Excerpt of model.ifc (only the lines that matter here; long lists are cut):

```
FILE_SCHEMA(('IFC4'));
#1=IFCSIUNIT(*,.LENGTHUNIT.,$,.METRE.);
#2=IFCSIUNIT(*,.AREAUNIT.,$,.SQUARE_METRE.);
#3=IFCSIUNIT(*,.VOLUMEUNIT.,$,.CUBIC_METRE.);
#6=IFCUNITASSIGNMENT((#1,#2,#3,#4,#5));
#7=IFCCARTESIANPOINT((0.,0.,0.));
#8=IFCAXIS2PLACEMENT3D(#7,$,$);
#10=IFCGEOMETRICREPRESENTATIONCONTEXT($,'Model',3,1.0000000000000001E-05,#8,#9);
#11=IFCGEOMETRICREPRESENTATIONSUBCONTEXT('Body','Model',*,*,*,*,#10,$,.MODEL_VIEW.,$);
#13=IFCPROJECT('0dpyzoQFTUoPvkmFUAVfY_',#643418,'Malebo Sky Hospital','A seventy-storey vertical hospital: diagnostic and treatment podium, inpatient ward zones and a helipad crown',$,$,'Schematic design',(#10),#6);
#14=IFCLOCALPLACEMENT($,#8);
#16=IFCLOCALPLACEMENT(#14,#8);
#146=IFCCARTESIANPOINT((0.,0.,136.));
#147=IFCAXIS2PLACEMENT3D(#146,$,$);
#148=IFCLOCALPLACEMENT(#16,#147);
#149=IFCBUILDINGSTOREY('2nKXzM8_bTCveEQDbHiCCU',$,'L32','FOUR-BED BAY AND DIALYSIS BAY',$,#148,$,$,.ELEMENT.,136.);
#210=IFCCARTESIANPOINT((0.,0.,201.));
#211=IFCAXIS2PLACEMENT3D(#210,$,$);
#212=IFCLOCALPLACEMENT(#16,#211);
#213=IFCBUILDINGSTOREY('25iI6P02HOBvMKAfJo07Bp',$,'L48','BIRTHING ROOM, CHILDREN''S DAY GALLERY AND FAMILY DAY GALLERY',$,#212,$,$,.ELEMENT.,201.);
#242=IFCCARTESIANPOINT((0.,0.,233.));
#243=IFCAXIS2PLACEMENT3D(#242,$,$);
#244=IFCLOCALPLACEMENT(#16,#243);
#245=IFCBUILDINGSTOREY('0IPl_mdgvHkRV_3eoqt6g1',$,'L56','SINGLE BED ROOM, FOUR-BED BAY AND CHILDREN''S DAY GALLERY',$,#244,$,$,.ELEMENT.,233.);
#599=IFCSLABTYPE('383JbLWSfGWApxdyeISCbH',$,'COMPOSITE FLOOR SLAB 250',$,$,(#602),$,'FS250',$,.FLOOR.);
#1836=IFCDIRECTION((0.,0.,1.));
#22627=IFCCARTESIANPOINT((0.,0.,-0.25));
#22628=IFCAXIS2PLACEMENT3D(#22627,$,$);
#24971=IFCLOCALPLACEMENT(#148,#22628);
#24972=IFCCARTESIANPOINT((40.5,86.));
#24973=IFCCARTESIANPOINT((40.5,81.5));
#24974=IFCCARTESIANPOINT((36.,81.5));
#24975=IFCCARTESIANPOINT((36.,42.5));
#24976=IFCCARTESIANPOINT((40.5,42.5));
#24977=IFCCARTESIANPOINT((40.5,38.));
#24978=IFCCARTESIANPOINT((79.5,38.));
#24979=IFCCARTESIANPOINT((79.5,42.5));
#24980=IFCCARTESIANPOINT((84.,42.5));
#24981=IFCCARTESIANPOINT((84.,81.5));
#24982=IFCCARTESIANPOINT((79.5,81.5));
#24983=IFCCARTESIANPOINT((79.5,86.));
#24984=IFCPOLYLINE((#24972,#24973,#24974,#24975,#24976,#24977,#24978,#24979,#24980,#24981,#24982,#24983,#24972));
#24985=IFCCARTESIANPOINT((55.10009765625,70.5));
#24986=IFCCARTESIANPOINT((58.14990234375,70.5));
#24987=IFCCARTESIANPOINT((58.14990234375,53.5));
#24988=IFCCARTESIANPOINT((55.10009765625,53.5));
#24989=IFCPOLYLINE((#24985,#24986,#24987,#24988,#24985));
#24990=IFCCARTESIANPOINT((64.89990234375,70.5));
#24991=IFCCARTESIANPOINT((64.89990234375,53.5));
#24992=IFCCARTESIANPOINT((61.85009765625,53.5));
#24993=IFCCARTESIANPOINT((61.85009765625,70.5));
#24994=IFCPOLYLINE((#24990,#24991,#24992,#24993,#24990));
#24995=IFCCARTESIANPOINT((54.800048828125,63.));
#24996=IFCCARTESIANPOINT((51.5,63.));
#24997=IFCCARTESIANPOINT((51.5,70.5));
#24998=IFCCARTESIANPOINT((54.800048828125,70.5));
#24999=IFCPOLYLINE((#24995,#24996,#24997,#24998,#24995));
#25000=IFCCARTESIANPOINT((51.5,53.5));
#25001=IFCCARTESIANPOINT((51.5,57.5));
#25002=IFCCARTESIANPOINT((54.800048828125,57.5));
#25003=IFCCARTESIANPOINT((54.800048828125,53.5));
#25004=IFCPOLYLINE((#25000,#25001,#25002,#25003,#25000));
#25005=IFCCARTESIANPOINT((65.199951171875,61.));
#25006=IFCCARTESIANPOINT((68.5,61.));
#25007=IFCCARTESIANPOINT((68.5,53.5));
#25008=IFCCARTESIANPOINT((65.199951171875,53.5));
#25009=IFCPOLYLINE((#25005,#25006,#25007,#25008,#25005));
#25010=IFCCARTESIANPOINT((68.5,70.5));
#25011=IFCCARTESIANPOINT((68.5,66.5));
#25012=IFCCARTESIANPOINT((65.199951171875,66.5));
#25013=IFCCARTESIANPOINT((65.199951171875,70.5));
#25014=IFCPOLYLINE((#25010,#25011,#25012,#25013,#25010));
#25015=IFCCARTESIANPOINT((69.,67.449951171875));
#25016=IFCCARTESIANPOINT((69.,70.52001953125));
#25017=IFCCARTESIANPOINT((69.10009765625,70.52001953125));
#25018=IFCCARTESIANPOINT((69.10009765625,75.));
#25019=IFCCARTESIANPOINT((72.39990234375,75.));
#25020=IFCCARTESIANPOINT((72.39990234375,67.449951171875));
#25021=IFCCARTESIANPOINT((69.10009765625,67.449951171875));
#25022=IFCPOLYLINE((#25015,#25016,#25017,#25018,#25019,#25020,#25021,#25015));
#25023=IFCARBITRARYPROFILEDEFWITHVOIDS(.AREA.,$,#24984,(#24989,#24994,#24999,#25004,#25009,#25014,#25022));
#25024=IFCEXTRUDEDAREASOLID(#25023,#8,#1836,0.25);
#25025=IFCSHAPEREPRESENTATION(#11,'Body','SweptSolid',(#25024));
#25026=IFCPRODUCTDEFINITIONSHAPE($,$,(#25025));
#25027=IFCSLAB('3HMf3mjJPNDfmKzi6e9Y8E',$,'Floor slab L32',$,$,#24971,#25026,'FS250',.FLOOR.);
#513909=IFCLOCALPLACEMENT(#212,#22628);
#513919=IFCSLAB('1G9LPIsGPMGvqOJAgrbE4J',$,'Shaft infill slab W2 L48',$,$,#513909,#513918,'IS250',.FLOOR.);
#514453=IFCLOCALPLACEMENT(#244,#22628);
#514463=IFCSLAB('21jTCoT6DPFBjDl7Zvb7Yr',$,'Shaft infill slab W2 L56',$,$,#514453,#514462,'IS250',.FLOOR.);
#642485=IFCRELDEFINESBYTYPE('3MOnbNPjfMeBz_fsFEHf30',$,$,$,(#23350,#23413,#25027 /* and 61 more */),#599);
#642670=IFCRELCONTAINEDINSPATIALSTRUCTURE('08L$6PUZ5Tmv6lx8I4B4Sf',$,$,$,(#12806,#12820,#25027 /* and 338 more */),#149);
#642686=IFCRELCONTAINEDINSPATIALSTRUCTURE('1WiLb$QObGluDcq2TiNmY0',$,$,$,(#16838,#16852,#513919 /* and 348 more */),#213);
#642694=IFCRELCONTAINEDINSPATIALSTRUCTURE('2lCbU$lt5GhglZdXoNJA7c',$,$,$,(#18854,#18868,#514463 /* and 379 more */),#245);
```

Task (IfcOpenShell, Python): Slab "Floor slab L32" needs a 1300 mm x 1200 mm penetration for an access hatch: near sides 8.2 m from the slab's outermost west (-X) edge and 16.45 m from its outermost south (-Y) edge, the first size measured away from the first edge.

```python
import numpy as np
import ifcopenshell
import ifcopenshell.api.feature
import ifcopenshell.api.geometry
import ifcopenshell.api.root
import ifcopenshell.geom
import ifcopenshell.util.placement
import ifcopenshell.util.representation
import ifcopenshell.util.shape
import ifcopenshell.util.unit

model = ifcopenshell.open("model.ifc")
unit_scale = ifcopenshell.util.unit.calculate_unit_scale(model)
settings = ifcopenshell.geom.settings()


def volume(element):
    """Net volume in cubic metres, openings subtracted."""
    shape = ifcopenshell.geom.create_shape(settings, element)
    return ifcopenshell.util.shape.get_volume(shape.geometry)


slab = model.by_guid("3HMf3mjJPNDfmKzi6e9Y8E")
before = volume(slab)

# Extent in the slab's own axes, in metres. The edges named are its -X and -Y sides.
slab_shape = ifcopenshell.geom.create_shape(settings, slab)
vertices = ifcopenshell.util.shape.get_vertices(slab_shape.geometry)
x_min, y_min, bottom = vertices.min(axis=0)
top = vertices[:, 2].max()

opening = ifcopenshell.api.root.create_entity(model, ifc_class="IfcOpeningElement", name="Access hatch opening", predefined_type="OPENING")
context = ifcopenshell.util.representation.get_context(model, "Model", "Body", "MODEL_VIEW")
width, depth = 1.3, 1.2
outline = [(0.0, 0.0), (width, 0.0), (width, depth), (0.0, depth), (0.0, 0.0)]
# Overshoot both faces by 50 mm so the cut is clean.
shape = ifcopenshell.api.geometry.add_slab_representation(
    model, context=context, depth=top - bottom + 0.1, polyline=outline
)
ifcopenshell.api.geometry.assign_representation(model, product=opening, representation=shape)

matrix = ifcopenshell.util.placement.get_local_placement(slab.ObjectPlacement)
matrix[:, 3] = matrix @ np.append(np.array([x_min + 8.2, y_min + 16.45, bottom - 0.05]) / unit_scale, 1.0)
ifcopenshell.api.geometry.edit_object_placement(model, product=opening, matrix=matrix, is_si=False)
ifcopenshell.api.feature.add_feature(model, feature=opening, element=slab)

after = volume(slab)

print(f"slab volume {before:.3f} -> {after:.3f} m3")

model.write("model-out.ifc")
```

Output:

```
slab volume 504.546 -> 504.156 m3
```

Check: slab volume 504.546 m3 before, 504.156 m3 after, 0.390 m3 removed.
